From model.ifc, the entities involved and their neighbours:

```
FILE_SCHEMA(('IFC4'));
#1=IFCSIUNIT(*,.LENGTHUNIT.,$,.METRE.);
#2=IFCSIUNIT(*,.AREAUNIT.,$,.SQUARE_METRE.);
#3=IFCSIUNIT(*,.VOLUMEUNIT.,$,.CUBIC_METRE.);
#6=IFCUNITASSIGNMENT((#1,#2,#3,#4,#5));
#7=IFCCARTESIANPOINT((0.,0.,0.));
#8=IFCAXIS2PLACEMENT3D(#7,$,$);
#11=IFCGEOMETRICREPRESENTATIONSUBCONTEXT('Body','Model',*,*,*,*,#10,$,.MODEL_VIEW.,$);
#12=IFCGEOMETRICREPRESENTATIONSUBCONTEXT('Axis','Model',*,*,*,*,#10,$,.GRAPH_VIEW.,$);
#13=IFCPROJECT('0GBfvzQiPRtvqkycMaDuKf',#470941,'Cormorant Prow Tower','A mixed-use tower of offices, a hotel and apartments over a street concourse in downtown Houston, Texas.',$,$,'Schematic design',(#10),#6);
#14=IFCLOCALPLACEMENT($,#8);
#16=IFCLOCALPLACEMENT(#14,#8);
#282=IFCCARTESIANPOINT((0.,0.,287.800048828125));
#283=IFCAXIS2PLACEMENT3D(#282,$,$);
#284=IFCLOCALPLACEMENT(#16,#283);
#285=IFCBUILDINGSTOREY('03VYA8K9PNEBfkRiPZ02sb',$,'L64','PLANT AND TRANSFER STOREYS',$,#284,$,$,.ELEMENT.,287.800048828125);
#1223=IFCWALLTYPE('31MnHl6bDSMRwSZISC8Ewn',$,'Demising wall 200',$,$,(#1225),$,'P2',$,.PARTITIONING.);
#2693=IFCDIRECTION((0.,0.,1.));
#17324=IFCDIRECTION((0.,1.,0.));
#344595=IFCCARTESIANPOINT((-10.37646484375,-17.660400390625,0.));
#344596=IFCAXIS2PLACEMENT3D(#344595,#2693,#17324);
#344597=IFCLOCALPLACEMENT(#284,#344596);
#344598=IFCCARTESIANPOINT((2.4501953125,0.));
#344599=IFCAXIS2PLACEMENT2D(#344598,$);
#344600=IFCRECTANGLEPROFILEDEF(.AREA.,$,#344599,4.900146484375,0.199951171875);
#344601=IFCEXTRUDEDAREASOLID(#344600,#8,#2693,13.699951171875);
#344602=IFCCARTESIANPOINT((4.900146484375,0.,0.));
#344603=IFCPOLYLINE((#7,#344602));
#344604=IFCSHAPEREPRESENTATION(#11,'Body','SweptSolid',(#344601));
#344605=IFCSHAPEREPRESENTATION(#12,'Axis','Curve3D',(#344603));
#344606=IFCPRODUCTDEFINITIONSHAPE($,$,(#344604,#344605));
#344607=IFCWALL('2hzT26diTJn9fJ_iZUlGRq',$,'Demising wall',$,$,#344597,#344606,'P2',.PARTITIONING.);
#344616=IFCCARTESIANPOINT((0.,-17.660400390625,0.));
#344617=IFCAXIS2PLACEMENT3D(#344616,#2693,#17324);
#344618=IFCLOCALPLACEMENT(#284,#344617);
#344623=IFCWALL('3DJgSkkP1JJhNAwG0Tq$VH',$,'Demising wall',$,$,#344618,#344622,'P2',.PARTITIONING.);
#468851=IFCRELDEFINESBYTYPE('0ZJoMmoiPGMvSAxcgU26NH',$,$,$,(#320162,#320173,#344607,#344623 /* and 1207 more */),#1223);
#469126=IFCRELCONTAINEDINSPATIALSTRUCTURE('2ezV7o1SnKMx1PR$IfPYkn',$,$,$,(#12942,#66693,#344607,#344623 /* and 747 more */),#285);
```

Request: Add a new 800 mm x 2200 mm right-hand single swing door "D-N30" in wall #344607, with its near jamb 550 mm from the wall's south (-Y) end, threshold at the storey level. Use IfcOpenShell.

```python
import numpy as np
import ifcopenshell
import ifcopenshell.api.feature
import ifcopenshell.api.geometry
import ifcopenshell.api.root
import ifcopenshell.api.spatial
import ifcopenshell.geom
import ifcopenshell.util.element
import ifcopenshell.util.placement
import ifcopenshell.util.representation
import ifcopenshell.util.shape
import ifcopenshell.util.unit

model = ifcopenshell.open("model.ifc")
unit_scale = ifcopenshell.util.unit.calculate_unit_scale(model)
settings = ifcopenshell.geom.settings()


def volume(element):
    """Net volume in cubic metres, openings subtracted."""
    shape = ifcopenshell.geom.create_shape(settings, element)
    return ifcopenshell.util.shape.get_volume(shape.geometry)


wall = model.by_guid("2hzT26diTJn9fJ_iZUlGRq")
storey = ifcopenshell.util.element.get_container(wall, ifc_class="IfcBuildingStorey")
context = ifcopenshell.util.representation.get_context(model, "Model", "Body", "MODEL_VIEW")
before = volume(wall)

width, height, from_end, sill = 0.8, 2.2, 0.55, 0.0  # metres

# The wall runs along its own X axis, and the end named is its -X end.
wall_shape = ifcopenshell.geom.create_shape(settings, wall)
x, y, z = ifcopenshell.util.shape.get_vertices(wall_shape.geometry).T
start = x.min() + from_end
face, thickness = float(y.min()), float(y.max() - y.min())
wall_matrix = ifcopenshell.util.placement.get_local_placement(wall.ObjectPlacement)
level = ifcopenshell.util.placement.get_local_placement(storey.ObjectPlacement)[2, 3]


def in_wall(x, y):
    """Placement at x, y metres in the wall's axes, at sill height."""
    matrix = wall_matrix.copy()
    matrix[:, 3] = wall_matrix @ np.array([x / unit_scale, y / unit_scale, 0.0, 1.0])
    matrix[2, 3] = level + sill / unit_scale
    return matrix


# Opening: a box that overshoots both wall faces by 50 mm.
opening = ifcopenshell.api.root.create_entity(model, ifc_class="IfcOpeningElement", predefined_type="OPENING")
box = ifcopenshell.api.geometry.add_wall_representation(
    model, context=context, length=width, height=height, thickness=thickness + 0.1
)
ifcopenshell.api.geometry.assign_representation(model, product=opening, representation=box)
ifcopenshell.api.geometry.edit_object_placement(model, product=opening, matrix=in_wall(start, face - 0.05), is_si=False)
ifcopenshell.api.feature.add_feature(model, feature=opening, element=wall)

door = ifcopenshell.api.root.create_entity(model, ifc_class="IfcDoor", name="D-N30", predefined_type="DOOR")
door.OverallWidth, door.OverallHeight = width / unit_scale, height / unit_scale
door.OperationType = "SINGLE_SWING_RIGHT"
body = ifcopenshell.api.geometry.add_door_representation(
    model,
    context=context,
    overall_width=door.OverallWidth,
    overall_height=door.OverallHeight,
    operation_type="SINGLE_SWING_RIGHT",
    lining_properties={"LiningDepth": thickness / unit_scale, "ThresholdDepth": thickness / unit_scale},
)
ifcopenshell.api.geometry.assign_representation(model, product=door, representation=body)
ifcopenshell.api.spatial.assign_container(model, products=[door], relating_structure=storey)
ifcopenshell.api.feature.add_filling(model, opening=opening, element=door)

# The lining spans the wall, so the door starts at the wall face.
ifcopenshell.api.geometry.edit_object_placement(model, product=door, matrix=in_wall(start, face), is_si=False)

after = volume(wall)

print(f"wall volume {before:.3f} -> {after:.3f} m3")

model.write("model_rev.ifc")
```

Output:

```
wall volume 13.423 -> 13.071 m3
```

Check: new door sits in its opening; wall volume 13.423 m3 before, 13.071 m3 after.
